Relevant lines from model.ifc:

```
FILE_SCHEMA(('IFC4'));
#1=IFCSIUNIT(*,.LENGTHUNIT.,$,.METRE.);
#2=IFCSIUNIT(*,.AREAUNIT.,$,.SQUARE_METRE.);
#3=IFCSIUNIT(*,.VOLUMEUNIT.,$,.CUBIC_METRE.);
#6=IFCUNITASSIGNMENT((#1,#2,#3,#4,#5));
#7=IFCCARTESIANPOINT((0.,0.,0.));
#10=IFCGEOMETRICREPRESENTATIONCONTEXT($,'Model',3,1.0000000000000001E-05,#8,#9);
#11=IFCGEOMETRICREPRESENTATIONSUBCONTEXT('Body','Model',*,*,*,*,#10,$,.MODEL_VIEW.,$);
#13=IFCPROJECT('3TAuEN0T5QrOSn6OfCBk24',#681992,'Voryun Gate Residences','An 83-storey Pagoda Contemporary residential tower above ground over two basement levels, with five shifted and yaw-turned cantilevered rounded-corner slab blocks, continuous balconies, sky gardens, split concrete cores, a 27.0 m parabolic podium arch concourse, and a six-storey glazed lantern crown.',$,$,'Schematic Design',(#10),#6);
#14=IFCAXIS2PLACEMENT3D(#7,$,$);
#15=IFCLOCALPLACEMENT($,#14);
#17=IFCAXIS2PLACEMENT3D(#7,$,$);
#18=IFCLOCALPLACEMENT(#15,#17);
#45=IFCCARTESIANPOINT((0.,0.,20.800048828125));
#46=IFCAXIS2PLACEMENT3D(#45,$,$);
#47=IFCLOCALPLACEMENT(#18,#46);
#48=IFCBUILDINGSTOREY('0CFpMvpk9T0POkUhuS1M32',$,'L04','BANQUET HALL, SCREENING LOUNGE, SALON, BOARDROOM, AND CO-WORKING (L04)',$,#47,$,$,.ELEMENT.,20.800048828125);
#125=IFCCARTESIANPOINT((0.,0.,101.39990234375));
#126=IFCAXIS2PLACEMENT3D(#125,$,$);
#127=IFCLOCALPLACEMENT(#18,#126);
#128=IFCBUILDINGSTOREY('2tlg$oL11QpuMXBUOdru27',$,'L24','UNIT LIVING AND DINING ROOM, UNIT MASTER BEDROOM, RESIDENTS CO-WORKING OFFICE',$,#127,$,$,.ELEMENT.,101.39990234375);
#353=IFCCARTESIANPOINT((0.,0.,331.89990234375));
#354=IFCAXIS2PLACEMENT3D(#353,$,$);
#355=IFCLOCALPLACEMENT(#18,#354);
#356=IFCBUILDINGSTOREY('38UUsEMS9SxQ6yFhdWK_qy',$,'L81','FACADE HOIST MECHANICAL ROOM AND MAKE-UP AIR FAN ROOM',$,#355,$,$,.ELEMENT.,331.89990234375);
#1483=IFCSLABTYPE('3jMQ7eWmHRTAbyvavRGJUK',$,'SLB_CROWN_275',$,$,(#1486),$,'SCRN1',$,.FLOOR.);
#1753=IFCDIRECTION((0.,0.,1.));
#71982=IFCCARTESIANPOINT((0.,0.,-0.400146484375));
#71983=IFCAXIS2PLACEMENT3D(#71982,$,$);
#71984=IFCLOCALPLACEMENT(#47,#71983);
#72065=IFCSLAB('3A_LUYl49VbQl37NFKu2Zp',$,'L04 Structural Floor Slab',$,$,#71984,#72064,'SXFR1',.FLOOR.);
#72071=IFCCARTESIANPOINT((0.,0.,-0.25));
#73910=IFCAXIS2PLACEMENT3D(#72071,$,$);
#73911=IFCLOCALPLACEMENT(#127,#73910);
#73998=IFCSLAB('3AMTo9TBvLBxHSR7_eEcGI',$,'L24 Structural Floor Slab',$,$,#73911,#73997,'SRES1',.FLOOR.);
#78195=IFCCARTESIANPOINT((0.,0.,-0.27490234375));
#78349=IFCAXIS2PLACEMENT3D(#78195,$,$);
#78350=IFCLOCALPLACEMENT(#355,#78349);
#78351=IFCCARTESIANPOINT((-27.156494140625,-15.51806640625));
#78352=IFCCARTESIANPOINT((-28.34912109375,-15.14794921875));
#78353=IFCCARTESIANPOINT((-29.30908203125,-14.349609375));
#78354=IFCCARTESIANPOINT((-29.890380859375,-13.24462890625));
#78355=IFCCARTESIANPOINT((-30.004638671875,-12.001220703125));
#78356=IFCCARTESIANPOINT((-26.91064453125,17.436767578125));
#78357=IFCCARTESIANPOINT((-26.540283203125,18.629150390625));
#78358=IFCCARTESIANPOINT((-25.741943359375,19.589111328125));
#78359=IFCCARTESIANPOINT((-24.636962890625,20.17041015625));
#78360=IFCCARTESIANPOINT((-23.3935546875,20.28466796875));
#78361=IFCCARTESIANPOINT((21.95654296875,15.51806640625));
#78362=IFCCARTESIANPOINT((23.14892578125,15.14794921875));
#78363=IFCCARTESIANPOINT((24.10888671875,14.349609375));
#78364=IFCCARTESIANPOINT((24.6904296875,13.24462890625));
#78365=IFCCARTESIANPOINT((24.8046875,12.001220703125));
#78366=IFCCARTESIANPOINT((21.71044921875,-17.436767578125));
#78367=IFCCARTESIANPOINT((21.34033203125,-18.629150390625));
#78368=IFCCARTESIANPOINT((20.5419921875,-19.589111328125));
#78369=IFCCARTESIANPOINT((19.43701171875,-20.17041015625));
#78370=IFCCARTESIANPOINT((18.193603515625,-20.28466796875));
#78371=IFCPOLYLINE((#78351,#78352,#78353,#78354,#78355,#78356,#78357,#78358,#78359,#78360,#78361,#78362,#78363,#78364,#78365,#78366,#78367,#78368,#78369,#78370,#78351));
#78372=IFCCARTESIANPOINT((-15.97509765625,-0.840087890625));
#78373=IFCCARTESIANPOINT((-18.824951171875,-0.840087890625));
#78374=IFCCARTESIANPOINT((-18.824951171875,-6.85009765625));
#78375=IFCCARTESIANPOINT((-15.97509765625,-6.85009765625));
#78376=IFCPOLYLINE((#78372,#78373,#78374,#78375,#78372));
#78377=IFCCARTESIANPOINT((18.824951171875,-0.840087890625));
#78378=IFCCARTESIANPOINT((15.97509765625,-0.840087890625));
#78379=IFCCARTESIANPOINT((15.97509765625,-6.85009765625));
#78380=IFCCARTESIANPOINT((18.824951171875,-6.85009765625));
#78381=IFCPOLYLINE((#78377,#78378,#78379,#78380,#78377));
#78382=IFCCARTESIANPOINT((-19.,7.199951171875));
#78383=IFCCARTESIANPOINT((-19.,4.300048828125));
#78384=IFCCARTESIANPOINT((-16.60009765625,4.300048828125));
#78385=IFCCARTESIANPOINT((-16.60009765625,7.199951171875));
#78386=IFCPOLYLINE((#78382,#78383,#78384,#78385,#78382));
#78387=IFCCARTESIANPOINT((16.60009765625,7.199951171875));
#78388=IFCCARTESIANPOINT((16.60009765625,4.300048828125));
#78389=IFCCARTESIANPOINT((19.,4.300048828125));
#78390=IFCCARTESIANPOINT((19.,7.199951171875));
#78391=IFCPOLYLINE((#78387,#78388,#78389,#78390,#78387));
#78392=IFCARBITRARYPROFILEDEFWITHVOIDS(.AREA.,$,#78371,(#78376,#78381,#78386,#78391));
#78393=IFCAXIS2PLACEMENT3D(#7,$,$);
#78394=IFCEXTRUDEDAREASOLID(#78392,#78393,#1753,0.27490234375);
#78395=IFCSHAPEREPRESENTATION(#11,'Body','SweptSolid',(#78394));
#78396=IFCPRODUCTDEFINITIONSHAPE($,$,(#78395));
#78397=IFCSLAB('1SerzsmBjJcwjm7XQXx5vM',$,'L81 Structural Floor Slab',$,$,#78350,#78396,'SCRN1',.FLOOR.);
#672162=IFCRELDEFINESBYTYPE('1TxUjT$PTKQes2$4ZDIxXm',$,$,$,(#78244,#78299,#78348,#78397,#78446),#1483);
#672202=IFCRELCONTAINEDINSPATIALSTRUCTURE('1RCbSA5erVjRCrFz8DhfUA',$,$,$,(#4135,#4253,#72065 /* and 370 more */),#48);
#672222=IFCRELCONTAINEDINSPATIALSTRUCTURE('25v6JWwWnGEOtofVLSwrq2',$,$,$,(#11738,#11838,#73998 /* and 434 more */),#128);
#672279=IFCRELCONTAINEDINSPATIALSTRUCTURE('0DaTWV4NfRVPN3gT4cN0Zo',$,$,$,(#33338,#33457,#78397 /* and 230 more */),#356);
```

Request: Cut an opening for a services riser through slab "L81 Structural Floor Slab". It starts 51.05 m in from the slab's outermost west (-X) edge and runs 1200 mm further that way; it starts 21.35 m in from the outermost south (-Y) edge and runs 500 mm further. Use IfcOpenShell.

```python
import numpy as np
import ifcopenshell
import ifcopenshell.api.feature
import ifcopenshell.api.geometry
import ifcopenshell.api.root
import ifcopenshell.geom
import ifcopenshell.util.placement
import ifcopenshell.util.representation
import ifcopenshell.util.shape
import ifcopenshell.util.unit

model = ifcopenshell.open("model.ifc")
unit_scale = ifcopenshell.util.unit.calculate_unit_scale(model)
settings = ifcopenshell.geom.settings()


def volume(element):
    """Net volume in cubic metres, openings subtracted."""
    shape = ifcopenshell.geom.create_shape(settings, element)
    return ifcopenshell.util.shape.get_volume(shape.geometry)


slab = model.by_id(78397)
before = volume(slab)

# Extent in the slab's own axes, in metres. The edges named are its -X and -Y sides.
slab_shape = ifcopenshell.geom.create_shape(settings, slab)
vertices = ifcopenshell.util.shape.get_vertices(slab_shape.geometry)
x_min, y_min, bottom = vertices.min(axis=0)
top = vertices[:, 2].max()

opening = ifcopenshell.api.root.create_entity(model, ifc_class="IfcOpeningElement", name="Services riser opening", predefined_type="OPENING")
context = ifcopenshell.util.representation.get_context(model, "Model", "Body", "MODEL_VIEW")
width, depth = 1.2, 0.5
outline = [(0.0, 0.0), (width, 0.0), (width, depth), (0.0, depth), (0.0, 0.0)]
# Overshoot both faces by 50 mm so the cut is clean.
shape = ifcopenshell.api.geometry.add_slab_representation(
    model, context=context, depth=top - bottom + 0.1, polyline=outline
)
ifcopenshell.api.geometry.assign_representation(model, product=opening, representation=shape)

matrix = ifcopenshell.util.placement.get_local_placement(slab.ObjectPlacement)
matrix[:, 3] = matrix @ np.append(np.array([x_min + 51.05, y_min + 21.35, bottom - 0.05]) / unit_scale, 1.0)
ifcopenshell.api.geometry.edit_object_placement(model, product=opening, matrix=matrix, is_si=False)
ifcopenshell.api.feature.add_feature(model, feature=opening, element=slab)

after = volume(slab)

print(f"slab volume {before:.3f} -> {after:.3f} m3")

model.write("model_v2.ifc")
```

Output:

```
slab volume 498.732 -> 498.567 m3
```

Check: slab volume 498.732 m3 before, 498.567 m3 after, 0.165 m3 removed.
